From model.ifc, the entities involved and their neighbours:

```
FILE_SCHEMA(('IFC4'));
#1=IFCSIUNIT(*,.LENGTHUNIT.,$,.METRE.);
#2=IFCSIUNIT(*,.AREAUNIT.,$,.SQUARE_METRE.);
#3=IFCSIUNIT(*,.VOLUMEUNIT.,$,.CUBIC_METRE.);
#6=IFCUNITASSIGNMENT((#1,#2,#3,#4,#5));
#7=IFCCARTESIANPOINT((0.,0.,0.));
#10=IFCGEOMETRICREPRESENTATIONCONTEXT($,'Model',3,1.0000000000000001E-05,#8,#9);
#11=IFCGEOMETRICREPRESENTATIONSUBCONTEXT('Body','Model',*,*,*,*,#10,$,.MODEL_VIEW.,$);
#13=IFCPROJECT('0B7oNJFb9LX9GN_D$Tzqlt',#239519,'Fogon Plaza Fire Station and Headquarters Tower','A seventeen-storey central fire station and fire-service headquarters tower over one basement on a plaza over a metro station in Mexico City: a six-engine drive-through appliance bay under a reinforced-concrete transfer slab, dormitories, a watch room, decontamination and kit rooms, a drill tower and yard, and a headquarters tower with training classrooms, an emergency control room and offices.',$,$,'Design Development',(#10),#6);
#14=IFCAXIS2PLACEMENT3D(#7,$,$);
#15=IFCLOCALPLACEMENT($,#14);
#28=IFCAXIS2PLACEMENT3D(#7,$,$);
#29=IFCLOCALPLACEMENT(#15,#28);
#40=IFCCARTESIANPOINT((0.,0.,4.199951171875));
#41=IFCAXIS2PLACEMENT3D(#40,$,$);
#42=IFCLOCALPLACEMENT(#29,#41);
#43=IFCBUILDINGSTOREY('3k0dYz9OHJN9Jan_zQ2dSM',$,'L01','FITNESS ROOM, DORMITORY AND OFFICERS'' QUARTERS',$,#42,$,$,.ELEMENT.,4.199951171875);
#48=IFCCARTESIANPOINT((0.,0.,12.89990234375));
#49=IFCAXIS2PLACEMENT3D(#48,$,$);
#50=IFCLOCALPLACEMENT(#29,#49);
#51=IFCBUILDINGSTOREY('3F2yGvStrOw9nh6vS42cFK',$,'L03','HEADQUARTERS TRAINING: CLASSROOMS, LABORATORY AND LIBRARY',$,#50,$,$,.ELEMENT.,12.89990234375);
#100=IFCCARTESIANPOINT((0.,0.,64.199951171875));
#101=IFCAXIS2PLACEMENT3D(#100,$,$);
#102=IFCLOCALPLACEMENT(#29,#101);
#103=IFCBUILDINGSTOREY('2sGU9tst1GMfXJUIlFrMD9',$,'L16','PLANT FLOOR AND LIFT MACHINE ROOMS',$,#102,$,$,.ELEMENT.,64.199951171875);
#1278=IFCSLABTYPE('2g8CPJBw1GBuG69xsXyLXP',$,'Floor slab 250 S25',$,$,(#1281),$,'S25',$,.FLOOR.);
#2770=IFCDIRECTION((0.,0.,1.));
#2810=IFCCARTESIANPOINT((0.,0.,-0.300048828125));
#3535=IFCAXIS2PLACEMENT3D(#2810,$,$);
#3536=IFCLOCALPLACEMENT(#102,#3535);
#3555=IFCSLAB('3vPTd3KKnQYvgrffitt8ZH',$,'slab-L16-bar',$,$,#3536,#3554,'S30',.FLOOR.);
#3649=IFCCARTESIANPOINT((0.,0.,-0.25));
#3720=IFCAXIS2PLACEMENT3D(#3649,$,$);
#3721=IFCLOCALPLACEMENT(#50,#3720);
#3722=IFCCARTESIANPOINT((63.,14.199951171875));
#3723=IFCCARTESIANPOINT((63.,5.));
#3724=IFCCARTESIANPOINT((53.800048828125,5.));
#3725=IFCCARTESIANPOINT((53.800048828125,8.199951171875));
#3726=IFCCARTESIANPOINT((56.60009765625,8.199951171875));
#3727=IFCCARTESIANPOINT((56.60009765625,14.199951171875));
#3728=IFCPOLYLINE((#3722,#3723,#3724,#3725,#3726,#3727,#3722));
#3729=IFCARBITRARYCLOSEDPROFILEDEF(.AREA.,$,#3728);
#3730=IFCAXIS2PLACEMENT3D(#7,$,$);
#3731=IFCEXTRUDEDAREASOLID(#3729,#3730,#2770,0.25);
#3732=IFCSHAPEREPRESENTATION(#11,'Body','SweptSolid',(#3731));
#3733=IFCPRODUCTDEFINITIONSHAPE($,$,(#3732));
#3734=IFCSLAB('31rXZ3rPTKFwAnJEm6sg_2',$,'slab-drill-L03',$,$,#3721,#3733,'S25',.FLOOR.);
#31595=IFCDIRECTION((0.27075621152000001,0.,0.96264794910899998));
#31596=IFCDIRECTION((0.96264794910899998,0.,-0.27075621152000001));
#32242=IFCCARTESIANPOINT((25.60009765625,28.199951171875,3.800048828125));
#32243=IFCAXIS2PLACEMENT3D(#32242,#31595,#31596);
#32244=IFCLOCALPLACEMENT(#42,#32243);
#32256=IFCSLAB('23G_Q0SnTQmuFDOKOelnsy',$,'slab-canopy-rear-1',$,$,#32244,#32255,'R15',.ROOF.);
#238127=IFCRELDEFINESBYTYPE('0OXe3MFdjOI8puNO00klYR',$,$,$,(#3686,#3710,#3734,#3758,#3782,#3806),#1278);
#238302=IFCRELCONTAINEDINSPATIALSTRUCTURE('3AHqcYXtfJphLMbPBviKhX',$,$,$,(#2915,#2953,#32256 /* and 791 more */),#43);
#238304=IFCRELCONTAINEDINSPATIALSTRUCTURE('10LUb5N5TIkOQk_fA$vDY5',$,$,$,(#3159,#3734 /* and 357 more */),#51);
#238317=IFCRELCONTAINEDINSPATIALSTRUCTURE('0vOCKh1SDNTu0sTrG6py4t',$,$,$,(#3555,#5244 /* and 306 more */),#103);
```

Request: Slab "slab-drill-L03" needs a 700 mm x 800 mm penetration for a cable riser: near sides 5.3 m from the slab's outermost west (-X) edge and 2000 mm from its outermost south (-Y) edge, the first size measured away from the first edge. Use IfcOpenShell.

```python
import numpy as np
import ifcopenshell
import ifcopenshell.api.feature
import ifcopenshell.api.geometry
import ifcopenshell.api.root
import ifcopenshell.geom
import ifcopenshell.util.placement
import ifcopenshell.util.representation
import ifcopenshell.util.shape
import ifcopenshell.util.unit

model = ifcopenshell.open("model.ifc")
unit_scale = ifcopenshell.util.unit.calculate_unit_scale(model)
settings = ifcopenshell.geom.settings()


def volume(element):
    """Net volume in cubic metres, openings subtracted."""
    shape = ifcopenshell.geom.create_shape(settings, element)
    return ifcopenshell.util.shape.get_volume(shape.geometry)


slab = model.by_id(3734)
before = volume(slab)

# Extent in the slab's own axes, in metres. The edges named are its -X and -Y sides.
slab_shape = ifcopenshell.geom.create_shape(settings, slab)
vertices = ifcopenshell.util.shape.get_vertices(slab_shape.geometry)
x_min, y_min, bottom = vertices.min(axis=0)
top = vertices[:, 2].max()

opening = ifcopenshell.api.root.create_entity(model, ifc_class="IfcOpeningElement", name="Cable riser opening", predefined_type="OPENING")
context = ifcopenshell.util.representation.get_context(model, "Model", "Body", "MODEL_VIEW")
width, depth = 0.7, 0.8
outline = [(0.0, 0.0), (width, 0.0), (width, depth), (0.0, depth), (0.0, 0.0)]
# Overshoot both faces by 50 mm so the cut is clean.
shape = ifcopenshell.api.geometry.add_slab_representation(
    model, context=context, depth=top - bottom + 0.1, polyline=outline
)
ifcopenshell.api.geometry.assign_representation(model, product=opening, representation=shape)

matrix = ifcopenshell.util.placement.get_local_placement(slab.ObjectPlacement)
matrix[:, 3] = matrix @ np.append(np.array([x_min + 5.3, y_min + 2, bottom - 0.05]) / unit_scale, 1.0)
ifcopenshell.api.geometry.edit_object_placement(model, product=opening, matrix=matrix, is_si=False)
ifcopenshell.api.feature.add_feature(model, feature=opening, element=slab)

after = volume(slab)

print(f"slab volume {before:.3f} -> {after:.3f} m3")

model.write("model_rev.ifc")
```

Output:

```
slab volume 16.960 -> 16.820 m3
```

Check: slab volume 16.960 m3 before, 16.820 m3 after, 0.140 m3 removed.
